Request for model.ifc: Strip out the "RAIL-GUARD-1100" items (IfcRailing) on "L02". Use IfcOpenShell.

First a look at what the model holds.

```python
import ifcopenshell
import ifcopenshell.util.element

model = ifcopenshell.open("model.ifc")
print(model.schema)
storey = next(s for s in model.by_type("IfcBuildingStorey") if s.Name == "L02")
railings = [e for e in ifcopenshell.util.element.get_decomposition(storey) if e.is_a("IfcRailing")]
seen = {}
for e in railings:
    element_type = ifcopenshell.util.element.get_type(e)
    name = element_type.Name if element_type not in (None, e) else None
    seen[name] = seen.get(name, 0) + 1
for name, count in sorted(seen.items(), key=str):
    print(count, "x", name)
```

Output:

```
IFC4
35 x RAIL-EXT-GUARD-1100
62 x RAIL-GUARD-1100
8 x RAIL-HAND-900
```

```python
import ifcopenshell
import ifcopenshell.api.root
import ifcopenshell.util.element

model = ifcopenshell.open("model.ifc")

storey = next(s for s in model.by_type("IfcBuildingStorey") if s.Name == "L02")
railings = [e for e in ifcopenshell.util.element.get_decomposition(storey) if e.is_a("IfcRailing")]
targets = [e for e in railings if (t := ifcopenshell.util.element.get_type(e)) not in (None, e) and t.Name == "RAIL-GUARD-1100"]

for e in targets:
    ifcopenshell.api.root.remove_product(model, product=e)
print(len(targets), "removed")

model.write("model_edited.ifc")
```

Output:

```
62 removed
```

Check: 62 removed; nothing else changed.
